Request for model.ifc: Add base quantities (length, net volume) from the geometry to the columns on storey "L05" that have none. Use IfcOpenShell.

First a look at what the model holds.

```python
import ifcopenshell
import ifcopenshell.util.element
import ifcopenshell.util.unit

model = ifcopenshell.open("model.ifc")
print(model.schema)
for unit_type in ("LENGTHUNIT", "AREAUNIT", "VOLUMEUNIT"):
    print(unit_type, ifcopenshell.util.unit.calculate_unit_scale(model, unit_type))
storey = next(s for s in model.by_type("IfcBuildingStorey") if s.Name == "L05")
columns = [e for e in ifcopenshell.util.element.get_decomposition(storey) if e.is_a("IfcColumn")]
for e in sorted(columns, key=lambda e: e.id()):
    print(e.id(), e.is_a(), e.Name, list(ifcopenshell.util.element.get_psets(e, qtos_only=True)), sep=" | ")
```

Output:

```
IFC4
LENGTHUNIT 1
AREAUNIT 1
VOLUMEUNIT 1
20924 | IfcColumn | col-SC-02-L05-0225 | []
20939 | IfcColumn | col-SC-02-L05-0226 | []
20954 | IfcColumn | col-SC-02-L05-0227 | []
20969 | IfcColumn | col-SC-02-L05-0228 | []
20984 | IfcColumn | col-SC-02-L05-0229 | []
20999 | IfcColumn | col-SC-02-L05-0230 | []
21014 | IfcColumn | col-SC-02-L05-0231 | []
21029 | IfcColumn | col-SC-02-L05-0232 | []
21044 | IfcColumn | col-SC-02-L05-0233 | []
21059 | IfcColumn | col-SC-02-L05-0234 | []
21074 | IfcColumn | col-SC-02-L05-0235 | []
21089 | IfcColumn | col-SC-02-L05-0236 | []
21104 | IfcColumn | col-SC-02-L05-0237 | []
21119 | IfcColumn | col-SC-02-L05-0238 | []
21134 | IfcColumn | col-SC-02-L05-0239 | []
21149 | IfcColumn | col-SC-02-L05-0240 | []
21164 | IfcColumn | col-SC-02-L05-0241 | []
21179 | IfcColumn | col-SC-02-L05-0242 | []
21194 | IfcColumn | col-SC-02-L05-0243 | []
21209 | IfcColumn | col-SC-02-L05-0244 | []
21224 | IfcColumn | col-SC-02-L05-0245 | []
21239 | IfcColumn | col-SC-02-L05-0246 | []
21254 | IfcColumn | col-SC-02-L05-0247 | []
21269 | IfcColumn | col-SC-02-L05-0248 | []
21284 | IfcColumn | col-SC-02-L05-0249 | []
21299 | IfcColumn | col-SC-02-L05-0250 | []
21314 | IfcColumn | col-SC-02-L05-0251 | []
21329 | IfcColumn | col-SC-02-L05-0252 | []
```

```python
import ifcopenshell
import ifcopenshell.api.pset
import ifcopenshell.geom
import ifcopenshell.util.element
import ifcopenshell.util.shape
import ifcopenshell.util.unit

model = ifcopenshell.open("model.ifc")
unit_scale = ifcopenshell.util.unit.calculate_unit_scale(model)
volume_scale = ifcopenshell.util.unit.calculate_unit_scale(model, "VOLUMEUNIT")
settings = ifcopenshell.geom.settings()

storey = next(s for s in model.by_type("IfcBuildingStorey") if s.Name == "L05")
columns = [e for e in ifcopenshell.util.element.get_decomposition(storey) if e.is_a("IfcColumn")]

for e in sorted(columns, key=lambda e: e.id()):
    if ifcopenshell.util.element.get_psets(e, qtos_only=True, should_inherit=False):
        continue
    # Geometry comes back in metres, in the element's own axes.
    shape = ifcopenshell.geom.create_shape(settings, e)
    values = {
        "Length": ifcopenshell.util.shape.get_z(shape.geometry) / unit_scale,
        "NetVolume": ifcopenshell.util.shape.get_volume(shape.geometry) / volume_scale,
    }
    qto = ifcopenshell.api.pset.add_qto(model, product=e, name="Qto_ColumnBaseQuantities")
    ifcopenshell.api.pset.edit_qto(model, qto=qto, properties=values)
    print(e.id(), {k: round(v, 3) for k, v in values.items()})

model.write("model-out.ifc")
```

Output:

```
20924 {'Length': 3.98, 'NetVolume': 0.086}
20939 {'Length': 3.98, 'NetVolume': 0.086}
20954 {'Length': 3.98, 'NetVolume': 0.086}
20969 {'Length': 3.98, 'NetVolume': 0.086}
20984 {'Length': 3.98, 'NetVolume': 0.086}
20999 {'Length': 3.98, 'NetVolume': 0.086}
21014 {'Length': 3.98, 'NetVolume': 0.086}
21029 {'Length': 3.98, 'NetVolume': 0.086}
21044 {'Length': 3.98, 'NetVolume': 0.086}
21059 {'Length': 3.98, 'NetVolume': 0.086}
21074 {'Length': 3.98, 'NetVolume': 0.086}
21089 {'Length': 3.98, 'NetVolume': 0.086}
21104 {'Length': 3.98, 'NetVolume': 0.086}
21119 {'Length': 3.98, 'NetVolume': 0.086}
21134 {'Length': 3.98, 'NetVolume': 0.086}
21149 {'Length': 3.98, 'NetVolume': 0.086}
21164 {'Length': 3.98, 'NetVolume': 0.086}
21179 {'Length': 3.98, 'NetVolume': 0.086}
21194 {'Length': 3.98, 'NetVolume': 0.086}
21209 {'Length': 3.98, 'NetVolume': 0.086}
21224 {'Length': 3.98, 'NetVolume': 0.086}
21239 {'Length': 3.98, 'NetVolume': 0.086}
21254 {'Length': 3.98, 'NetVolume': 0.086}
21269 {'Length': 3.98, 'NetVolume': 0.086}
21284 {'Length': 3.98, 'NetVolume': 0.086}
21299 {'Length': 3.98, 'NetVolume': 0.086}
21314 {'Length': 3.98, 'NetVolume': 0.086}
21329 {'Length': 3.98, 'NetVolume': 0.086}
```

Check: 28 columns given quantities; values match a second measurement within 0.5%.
